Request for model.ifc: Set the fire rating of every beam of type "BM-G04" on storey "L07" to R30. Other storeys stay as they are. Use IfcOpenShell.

First a look at what the model holds.

```python
import ifcopenshell
import ifcopenshell.util.element

model = ifcopenshell.open("model.ifc")
print(model.schema)
storey = next(s for s in model.by_type("IfcBuildingStorey") if s.Name == "L07")
beams = [e for e in ifcopenshell.util.element.get_decomposition(storey) if e.is_a("IfcBeam")]
seen = {}
for e in beams:
    element_type = ifcopenshell.util.element.get_type(e)
    key = (element_type.Name if element_type != e and element_type else None, ifcopenshell.util.element.get_pset(e, "Pset_BeamCommon", "FireRating"))
    seen[key] = seen.get(key, 0) + 1
for (name, value), count in sorted(seen.items(), key=str):
    print(count, "x", name, "|", value)
```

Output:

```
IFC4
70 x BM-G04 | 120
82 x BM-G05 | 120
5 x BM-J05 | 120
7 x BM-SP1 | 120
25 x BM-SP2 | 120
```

```python
import ifcopenshell
import ifcopenshell.api.pset
import ifcopenshell.util.element

model = ifcopenshell.open("model.ifc")

storey = next(s for s in model.by_type("IfcBuildingStorey") if s.Name == "L07")
beams = [e for e in ifcopenshell.util.element.get_decomposition(storey) if e.is_a("IfcBeam")]

count = 0
for e in beams:
    element_type = ifcopenshell.util.element.get_type(e)
    if element_type in (None, e) or element_type.Name != "BM-G04":
        continue
    # add_pset returns the element's existing set when there is one.
    pset = ifcopenshell.api.pset.add_pset(model, product=e, name="Pset_BeamCommon")
    ifcopenshell.api.pset.edit_pset(model, pset=pset, properties={"FireRating": "R30"})
    count += 1

print(count, "beams updated")

model.write("model_rev.ifc")
```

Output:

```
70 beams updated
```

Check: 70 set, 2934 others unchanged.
